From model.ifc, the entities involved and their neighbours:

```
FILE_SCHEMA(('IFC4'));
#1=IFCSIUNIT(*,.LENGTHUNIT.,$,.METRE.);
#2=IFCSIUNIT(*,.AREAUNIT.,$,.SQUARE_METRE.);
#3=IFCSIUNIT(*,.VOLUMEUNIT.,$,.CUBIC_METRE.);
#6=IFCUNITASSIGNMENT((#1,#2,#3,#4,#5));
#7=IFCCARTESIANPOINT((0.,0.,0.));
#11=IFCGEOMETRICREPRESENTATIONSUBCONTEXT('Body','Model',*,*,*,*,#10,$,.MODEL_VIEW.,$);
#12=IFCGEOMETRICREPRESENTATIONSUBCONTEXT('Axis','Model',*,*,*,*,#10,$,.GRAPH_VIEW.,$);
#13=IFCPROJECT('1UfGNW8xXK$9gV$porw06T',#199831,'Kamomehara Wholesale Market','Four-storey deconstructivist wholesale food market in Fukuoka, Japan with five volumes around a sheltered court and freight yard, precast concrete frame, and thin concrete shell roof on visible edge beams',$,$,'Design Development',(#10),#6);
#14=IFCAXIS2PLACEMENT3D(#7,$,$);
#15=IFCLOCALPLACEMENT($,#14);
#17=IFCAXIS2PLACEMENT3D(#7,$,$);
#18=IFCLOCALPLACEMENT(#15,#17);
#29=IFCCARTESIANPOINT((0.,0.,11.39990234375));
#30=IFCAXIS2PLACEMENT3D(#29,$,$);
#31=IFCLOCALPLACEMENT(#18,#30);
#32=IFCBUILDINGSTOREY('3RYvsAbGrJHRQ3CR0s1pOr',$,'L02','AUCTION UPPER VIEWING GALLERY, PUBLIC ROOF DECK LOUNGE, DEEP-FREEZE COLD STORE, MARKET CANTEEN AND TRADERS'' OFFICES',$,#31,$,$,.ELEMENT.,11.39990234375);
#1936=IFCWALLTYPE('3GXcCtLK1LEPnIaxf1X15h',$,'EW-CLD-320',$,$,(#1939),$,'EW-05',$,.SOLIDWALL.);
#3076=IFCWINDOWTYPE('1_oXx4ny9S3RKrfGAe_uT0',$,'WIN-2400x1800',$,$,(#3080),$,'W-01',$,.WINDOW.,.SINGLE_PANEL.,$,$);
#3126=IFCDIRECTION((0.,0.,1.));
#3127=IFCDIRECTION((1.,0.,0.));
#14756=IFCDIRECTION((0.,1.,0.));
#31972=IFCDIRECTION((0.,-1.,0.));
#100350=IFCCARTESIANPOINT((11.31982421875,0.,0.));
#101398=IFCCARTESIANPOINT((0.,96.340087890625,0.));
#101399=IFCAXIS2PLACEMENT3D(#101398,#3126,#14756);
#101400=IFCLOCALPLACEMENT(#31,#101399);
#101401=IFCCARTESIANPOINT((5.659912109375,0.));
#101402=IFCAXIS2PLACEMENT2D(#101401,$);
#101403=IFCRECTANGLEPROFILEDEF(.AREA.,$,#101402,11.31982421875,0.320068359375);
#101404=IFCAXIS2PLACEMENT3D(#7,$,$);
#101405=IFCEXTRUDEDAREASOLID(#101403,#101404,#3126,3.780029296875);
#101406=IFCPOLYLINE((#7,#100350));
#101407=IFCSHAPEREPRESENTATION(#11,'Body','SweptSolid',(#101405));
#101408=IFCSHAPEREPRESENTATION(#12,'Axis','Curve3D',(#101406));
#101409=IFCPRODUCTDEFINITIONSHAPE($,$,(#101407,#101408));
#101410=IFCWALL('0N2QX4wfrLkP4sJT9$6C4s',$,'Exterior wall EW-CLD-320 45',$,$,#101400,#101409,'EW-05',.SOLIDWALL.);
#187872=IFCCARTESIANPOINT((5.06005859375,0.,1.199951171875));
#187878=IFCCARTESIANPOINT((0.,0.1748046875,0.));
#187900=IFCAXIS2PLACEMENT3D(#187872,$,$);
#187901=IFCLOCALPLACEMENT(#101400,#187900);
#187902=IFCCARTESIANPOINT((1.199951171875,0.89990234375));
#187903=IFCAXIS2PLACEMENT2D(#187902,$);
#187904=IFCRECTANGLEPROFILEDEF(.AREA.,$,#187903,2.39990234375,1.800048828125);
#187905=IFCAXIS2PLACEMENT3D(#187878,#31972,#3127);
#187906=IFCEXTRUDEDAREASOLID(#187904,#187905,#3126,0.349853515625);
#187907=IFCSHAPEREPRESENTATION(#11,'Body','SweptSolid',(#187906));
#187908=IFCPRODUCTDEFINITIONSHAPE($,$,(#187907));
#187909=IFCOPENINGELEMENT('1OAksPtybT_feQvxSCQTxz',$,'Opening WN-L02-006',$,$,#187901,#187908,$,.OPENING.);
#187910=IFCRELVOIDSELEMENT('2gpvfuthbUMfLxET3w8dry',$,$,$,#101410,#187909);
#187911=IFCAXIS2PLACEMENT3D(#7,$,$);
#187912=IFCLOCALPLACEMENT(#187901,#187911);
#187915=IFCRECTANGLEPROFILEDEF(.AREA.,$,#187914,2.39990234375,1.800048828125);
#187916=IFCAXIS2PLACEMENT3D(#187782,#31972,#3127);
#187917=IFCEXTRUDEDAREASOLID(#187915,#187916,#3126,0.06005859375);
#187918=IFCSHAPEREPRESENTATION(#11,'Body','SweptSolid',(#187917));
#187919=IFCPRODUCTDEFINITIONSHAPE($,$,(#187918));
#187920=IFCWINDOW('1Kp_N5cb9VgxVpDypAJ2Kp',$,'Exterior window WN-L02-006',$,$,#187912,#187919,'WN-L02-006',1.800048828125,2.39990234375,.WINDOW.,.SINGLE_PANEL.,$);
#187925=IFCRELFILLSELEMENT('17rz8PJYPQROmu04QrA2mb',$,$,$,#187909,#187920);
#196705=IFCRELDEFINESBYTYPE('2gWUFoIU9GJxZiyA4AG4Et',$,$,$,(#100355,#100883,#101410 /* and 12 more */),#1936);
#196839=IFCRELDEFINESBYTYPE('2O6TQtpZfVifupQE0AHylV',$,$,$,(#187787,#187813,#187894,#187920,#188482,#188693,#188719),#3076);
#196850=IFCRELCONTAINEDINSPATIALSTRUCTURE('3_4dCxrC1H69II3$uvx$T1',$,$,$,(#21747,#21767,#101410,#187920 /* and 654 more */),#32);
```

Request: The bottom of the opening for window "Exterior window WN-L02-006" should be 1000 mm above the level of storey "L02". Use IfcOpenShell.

```python
import numpy as np
import ifcopenshell
import ifcopenshell.api.geometry
import ifcopenshell.geom
import ifcopenshell.util.element
import ifcopenshell.util.placement
import ifcopenshell.util.shape
import ifcopenshell.util.unit

model = ifcopenshell.open("model.ifc")
unit_scale = ifcopenshell.util.unit.calculate_unit_scale(model)

window = model.by_id(187920)
opening = window.FillsVoids[0].RelatingOpeningElement
storey = ifcopenshell.util.element.get_container(window, ifc_class="IfcBuildingStorey")
level = ifcopenshell.util.placement.get_local_placement(storey.ObjectPlacement)[2, 3]

# The opening's origin need not be at the sill, so measure its lowest point.
shape = ifcopenshell.geom.create_shape(ifcopenshell.geom.settings(), opening)
bottom = ifcopenshell.util.shape.get_shape_bottom_elevation(shape, shape.geometry) / unit_scale
dz = level + 1.0 - bottom

shift = np.array([0.0, 0.0, dz])
# The window is placed relative to its opening, so it follows when the opening moves.
matrix = ifcopenshell.util.placement.get_local_placement(opening.ObjectPlacement)
matrix[:3, 3] += shift
ifcopenshell.api.geometry.edit_object_placement(
    model, product=opening, matrix=matrix, is_si=False, should_transform_children=True
)

print(f"moved by {dz * unit_scale:+.3f} m")

model.write("model_rev.ifc")
```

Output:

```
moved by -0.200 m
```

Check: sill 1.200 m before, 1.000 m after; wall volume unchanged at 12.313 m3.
